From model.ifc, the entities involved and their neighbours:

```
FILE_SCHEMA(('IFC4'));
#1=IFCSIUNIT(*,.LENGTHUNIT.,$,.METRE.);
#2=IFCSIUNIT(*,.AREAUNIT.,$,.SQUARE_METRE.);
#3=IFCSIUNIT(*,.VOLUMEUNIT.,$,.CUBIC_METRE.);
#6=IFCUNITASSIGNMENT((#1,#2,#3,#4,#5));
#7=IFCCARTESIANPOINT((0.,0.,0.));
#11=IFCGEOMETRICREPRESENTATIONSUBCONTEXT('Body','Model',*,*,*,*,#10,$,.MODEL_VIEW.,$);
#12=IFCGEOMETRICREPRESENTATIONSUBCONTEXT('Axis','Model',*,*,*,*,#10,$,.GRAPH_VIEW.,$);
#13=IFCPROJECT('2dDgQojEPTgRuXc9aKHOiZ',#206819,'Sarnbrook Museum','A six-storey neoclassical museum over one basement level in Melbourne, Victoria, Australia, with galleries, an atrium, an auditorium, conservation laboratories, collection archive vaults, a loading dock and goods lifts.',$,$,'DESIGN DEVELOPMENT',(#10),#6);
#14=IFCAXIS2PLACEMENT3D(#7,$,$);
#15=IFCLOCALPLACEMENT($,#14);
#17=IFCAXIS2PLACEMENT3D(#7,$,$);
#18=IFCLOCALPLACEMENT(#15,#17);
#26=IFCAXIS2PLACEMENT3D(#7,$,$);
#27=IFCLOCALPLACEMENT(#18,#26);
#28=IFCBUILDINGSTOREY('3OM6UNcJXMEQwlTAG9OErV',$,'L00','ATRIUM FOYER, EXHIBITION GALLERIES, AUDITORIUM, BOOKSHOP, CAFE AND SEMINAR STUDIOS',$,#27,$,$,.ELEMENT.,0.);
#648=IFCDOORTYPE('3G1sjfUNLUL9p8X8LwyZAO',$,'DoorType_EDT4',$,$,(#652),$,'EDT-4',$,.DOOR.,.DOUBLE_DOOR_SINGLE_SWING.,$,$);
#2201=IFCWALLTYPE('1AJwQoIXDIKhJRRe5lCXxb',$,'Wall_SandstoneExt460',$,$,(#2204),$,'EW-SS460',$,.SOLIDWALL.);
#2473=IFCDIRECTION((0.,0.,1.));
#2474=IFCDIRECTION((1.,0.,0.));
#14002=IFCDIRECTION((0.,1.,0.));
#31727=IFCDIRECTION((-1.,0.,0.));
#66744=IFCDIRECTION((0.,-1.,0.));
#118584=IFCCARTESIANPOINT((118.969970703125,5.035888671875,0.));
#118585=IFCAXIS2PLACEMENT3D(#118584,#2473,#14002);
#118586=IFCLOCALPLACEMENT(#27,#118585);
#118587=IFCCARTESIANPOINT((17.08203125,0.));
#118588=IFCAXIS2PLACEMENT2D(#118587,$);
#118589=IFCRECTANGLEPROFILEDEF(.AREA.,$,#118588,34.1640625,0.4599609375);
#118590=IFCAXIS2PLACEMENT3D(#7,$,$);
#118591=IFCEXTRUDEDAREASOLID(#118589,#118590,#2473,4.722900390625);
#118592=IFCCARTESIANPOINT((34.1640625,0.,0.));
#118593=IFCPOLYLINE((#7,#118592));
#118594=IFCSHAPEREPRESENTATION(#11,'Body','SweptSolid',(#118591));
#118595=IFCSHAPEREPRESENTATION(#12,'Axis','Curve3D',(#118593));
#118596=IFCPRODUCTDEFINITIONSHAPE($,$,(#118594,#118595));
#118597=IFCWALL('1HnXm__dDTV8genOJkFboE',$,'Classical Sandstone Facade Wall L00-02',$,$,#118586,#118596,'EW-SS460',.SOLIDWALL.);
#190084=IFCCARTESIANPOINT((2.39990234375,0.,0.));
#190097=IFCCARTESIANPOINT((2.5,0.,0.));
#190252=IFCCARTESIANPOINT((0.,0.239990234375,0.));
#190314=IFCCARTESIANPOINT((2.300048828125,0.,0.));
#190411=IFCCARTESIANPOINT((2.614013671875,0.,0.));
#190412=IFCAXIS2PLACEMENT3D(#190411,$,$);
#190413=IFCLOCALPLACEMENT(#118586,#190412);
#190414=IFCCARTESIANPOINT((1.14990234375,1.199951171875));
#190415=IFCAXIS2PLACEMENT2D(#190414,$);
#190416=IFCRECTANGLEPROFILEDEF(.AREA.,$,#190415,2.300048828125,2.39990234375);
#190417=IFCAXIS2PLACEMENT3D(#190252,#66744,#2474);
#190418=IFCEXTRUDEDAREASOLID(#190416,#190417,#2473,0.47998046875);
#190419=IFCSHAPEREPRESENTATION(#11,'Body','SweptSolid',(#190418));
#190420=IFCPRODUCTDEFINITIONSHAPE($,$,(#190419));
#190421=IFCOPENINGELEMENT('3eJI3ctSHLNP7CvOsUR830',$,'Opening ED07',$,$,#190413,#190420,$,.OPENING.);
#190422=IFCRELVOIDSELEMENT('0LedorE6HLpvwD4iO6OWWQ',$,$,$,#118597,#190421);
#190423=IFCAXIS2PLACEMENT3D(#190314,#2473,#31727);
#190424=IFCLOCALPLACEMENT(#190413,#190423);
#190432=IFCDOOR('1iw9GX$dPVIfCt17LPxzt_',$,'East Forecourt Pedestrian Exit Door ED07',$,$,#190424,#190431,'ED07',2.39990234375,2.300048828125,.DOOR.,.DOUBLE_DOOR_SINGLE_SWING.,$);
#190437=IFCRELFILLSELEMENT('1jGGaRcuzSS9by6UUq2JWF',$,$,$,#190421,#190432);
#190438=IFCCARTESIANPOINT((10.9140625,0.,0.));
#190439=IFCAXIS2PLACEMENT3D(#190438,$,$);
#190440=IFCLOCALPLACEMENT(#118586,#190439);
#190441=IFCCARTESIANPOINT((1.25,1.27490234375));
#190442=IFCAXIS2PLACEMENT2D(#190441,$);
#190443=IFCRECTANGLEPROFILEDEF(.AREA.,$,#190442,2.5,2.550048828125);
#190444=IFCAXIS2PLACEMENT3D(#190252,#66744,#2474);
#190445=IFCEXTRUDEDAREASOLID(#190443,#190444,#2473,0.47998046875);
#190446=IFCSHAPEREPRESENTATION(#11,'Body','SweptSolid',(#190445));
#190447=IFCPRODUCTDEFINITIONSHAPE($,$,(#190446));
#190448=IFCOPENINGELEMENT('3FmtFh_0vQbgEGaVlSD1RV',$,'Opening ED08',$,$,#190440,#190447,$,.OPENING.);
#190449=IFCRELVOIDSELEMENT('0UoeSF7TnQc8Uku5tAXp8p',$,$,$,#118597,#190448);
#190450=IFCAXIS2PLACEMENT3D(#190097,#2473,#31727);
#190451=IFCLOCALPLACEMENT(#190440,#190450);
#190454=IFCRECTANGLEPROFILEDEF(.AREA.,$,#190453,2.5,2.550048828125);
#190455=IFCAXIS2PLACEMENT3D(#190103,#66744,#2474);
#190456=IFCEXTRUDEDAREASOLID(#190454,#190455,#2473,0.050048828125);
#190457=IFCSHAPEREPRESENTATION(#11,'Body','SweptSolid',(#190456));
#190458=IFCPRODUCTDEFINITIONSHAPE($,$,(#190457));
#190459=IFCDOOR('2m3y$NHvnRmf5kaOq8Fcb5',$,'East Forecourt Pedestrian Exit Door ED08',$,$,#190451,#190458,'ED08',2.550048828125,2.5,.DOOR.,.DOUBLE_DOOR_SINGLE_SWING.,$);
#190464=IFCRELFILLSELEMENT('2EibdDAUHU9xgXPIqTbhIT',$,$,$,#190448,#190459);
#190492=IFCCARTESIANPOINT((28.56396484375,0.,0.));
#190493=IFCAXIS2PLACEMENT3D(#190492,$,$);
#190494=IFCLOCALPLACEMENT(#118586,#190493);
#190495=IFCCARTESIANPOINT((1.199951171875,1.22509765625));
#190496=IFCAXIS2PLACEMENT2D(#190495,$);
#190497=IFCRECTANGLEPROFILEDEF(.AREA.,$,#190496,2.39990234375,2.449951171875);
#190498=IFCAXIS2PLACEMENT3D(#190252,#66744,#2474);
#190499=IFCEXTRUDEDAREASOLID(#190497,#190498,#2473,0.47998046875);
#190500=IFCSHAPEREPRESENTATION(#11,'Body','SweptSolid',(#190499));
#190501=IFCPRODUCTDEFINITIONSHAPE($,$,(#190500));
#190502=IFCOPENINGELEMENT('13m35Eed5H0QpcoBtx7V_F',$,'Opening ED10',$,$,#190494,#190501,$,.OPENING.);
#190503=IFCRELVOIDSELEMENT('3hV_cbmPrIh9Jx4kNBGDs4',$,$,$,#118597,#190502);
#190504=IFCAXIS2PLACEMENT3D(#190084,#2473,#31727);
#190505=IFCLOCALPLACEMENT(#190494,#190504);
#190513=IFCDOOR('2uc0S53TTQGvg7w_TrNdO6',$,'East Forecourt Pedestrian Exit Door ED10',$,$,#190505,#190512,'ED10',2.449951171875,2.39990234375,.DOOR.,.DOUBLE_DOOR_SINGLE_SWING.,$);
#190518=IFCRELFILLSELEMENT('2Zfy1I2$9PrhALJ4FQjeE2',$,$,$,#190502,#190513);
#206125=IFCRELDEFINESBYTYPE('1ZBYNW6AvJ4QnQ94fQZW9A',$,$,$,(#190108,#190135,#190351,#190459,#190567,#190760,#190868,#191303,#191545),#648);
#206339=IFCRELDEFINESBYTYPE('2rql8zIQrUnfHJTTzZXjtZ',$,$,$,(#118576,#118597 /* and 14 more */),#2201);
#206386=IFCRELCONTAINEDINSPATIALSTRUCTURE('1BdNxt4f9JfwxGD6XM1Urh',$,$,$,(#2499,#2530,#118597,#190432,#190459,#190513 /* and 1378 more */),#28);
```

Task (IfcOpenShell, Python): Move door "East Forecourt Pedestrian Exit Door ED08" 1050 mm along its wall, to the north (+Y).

```python
import ifcopenshell
import ifcopenshell.api.geometry
import ifcopenshell.util.placement

model = ifcopenshell.open("model.ifc")

door = model.by_guid("2m3y$NHvnRmf5kaOq8Fcb5")
opening = door.FillsVoids[0].RelatingOpeningElement
wall = opening.VoidsElements[0].RelatingBuildingElement

wall_matrix = ifcopenshell.util.placement.get_local_placement(wall.ObjectPlacement)
shift = wall_matrix[:3, 0] * 1.05
before = ifcopenshell.util.placement.get_local_placement(door.ObjectPlacement)[:3, 3].copy()

# The door is placed relative to its opening, so it follows when the opening moves.
matrix = ifcopenshell.util.placement.get_local_placement(opening.ObjectPlacement)
matrix[:3, 3] += shift
ifcopenshell.api.geometry.edit_object_placement(
    model, product=opening, matrix=matrix, is_si=False, should_transform_children=True
)

after = ifcopenshell.util.placement.get_local_placement(door.ObjectPlacement)[:3, 3]
print("door moved by", (after - before).round(3) + 0.0)

model.write("model_updated.ifc")
```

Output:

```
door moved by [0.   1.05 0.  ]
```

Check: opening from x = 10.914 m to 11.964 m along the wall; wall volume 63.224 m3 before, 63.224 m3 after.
